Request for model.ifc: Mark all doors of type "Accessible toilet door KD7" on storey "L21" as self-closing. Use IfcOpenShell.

First a look at what the model holds.

```python
import ifcopenshell
import ifcopenshell.util.element

model = ifcopenshell.open("model.ifc")
print(model.schema)
storey = next(s for s in model.by_type("IfcBuildingStorey") if s.Name == "L21")
doors = [e for e in ifcopenshell.util.element.get_decomposition(storey) if e.is_a("IfcDoor")]
seen = {}
for e in doors:
    element_type = ifcopenshell.util.element.get_type(e)
    key = (element_type.Name if element_type != e and element_type else None, ifcopenshell.util.element.get_pset(e, "Pset_DoorCommon", "SelfClosing"))
    seen[key] = seen.get(key, 0) + 1
for (name, value), count in sorted(seen.items(), key=str):
    print(count, "x", name, "|", value)
```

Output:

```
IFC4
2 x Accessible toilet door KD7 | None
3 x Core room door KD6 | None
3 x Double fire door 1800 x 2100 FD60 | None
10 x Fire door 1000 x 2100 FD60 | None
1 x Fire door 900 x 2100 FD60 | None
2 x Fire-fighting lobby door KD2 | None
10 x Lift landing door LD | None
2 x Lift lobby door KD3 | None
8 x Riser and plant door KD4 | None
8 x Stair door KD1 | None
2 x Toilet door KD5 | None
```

```python
import ifcopenshell
import ifcopenshell.api.pset
import ifcopenshell.util.element

model = ifcopenshell.open("model.ifc")

storey = next(s for s in model.by_type("IfcBuildingStorey") if s.Name == "L21")
doors = [e for e in ifcopenshell.util.element.get_decomposition(storey) if e.is_a("IfcDoor")]

count = 0
for e in doors:
    element_type = ifcopenshell.util.element.get_type(e)
    if element_type in (None, e) or element_type.Name != "Accessible toilet door KD7":
        continue
    found = ifcopenshell.util.element.get_pset(e, "Pset_DoorCommon", should_inherit=False)
    if found:
        pset = model.by_id(found["id"])
        if len(ifcopenshell.util.element.get_elements_by_pset(pset)) > 1:
            pset = ifcopenshell.api.pset.unshare_pset(model, products=[e], pset=pset)[0]
    else:
        pset = ifcopenshell.api.pset.add_pset(model, product=e, name="Pset_DoorCommon")
    ifcopenshell.api.pset.edit_pset(model, pset=pset, properties={"SelfClosing": True})
    count += 1

print(count, "doors updated")

model.write("model-out.ifc")
```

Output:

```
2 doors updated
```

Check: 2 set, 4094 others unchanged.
